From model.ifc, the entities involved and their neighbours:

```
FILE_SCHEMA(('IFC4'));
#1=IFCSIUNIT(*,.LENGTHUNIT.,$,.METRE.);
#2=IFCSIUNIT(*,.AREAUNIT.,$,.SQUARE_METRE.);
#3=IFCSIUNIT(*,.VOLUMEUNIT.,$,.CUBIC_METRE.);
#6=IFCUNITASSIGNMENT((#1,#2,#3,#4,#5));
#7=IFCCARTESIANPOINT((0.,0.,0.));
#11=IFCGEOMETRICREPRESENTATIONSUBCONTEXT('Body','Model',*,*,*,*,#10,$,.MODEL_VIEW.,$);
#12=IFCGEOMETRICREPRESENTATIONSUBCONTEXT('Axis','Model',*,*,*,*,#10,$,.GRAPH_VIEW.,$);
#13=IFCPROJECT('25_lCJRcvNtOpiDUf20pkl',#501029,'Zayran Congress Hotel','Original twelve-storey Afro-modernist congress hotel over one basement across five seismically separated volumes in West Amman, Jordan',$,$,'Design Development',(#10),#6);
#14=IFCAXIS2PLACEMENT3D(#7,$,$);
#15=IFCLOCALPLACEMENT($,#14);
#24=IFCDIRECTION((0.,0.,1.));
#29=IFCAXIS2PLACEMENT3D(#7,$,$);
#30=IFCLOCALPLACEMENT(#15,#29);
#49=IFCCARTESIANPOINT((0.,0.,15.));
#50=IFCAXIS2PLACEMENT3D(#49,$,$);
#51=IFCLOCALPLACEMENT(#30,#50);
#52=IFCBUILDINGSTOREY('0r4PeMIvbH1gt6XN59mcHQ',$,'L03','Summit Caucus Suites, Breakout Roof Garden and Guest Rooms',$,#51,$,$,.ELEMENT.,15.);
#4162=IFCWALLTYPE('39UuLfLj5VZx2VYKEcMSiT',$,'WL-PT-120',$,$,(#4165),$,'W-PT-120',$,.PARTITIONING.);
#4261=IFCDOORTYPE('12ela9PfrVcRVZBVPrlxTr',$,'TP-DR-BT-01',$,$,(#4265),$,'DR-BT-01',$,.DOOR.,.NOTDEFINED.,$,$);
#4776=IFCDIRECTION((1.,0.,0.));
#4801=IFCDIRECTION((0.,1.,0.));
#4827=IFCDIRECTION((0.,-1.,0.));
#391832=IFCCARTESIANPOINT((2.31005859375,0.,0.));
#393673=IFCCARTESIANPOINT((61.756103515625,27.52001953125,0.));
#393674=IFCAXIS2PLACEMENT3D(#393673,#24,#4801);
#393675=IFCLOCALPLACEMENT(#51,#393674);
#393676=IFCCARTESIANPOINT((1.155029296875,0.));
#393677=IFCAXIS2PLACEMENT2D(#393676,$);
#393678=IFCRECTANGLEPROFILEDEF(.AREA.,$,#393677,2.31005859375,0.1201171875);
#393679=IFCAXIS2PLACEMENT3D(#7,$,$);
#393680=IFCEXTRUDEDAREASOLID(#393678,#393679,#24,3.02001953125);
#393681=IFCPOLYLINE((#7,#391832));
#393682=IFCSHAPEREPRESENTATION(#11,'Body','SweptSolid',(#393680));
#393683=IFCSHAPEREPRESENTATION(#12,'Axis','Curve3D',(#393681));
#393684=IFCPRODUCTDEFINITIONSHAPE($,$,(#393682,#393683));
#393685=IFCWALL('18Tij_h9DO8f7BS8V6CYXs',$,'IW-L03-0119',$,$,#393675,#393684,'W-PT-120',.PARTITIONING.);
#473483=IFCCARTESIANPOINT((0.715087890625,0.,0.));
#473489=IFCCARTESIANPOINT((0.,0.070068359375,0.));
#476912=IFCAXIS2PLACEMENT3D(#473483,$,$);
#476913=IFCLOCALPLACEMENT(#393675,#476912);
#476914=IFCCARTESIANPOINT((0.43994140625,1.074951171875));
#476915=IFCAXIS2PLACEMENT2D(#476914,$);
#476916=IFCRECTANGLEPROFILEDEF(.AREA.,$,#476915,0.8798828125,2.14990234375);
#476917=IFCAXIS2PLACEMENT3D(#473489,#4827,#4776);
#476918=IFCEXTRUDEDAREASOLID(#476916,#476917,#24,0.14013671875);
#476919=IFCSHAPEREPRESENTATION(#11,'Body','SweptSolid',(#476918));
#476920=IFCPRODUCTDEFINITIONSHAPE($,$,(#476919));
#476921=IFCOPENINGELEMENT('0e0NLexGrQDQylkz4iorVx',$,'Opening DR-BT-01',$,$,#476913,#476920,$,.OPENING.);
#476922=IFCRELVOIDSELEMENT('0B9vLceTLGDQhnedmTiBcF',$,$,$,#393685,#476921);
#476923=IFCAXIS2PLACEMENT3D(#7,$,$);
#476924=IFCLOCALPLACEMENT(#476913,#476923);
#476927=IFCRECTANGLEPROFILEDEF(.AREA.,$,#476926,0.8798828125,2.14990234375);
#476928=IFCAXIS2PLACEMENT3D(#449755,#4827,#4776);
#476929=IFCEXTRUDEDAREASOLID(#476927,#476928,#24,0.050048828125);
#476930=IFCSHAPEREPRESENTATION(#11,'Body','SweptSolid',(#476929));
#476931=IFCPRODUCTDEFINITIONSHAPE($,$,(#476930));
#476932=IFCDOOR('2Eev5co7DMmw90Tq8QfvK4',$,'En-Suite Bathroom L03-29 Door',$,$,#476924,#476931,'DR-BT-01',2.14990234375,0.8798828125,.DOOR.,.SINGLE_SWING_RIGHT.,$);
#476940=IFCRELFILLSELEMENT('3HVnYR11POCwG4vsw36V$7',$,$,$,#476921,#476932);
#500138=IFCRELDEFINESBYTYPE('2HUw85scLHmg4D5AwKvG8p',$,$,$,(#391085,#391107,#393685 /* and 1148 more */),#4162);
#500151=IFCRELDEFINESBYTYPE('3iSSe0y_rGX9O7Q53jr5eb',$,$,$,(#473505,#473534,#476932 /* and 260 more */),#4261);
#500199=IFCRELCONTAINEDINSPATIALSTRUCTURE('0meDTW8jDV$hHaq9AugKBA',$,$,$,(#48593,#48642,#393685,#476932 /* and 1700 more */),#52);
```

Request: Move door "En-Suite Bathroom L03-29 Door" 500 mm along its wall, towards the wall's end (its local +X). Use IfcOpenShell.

```python
import ifcopenshell
import ifcopenshell.api.geometry
import ifcopenshell.util.placement

model = ifcopenshell.open("model.ifc")

door = model.by_guid("2Eev5co7DMmw90Tq8QfvK4")
opening = door.FillsVoids[0].RelatingOpeningElement
wall = opening.VoidsElements[0].RelatingBuildingElement

wall_matrix = ifcopenshell.util.placement.get_local_placement(wall.ObjectPlacement)
shift = wall_matrix[:3, 0] * 0.5
before = ifcopenshell.util.placement.get_local_placement(door.ObjectPlacement)[:3, 3].copy()

# The door is placed relative to its opening, so it follows when the opening moves.
matrix = ifcopenshell.util.placement.get_local_placement(opening.ObjectPlacement)
matrix[:3, 3] += shift
ifcopenshell.api.geometry.edit_object_placement(
    model, product=opening, matrix=matrix, is_si=False, should_transform_children=True
)

after = ifcopenshell.util.placement.get_local_placement(door.ObjectPlacement)[:3, 3]
print("door moved by", (after - before).round(3) + 0.0)

model.write("model_v2.ifc")
```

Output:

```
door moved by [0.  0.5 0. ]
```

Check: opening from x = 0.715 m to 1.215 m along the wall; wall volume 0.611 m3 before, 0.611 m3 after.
